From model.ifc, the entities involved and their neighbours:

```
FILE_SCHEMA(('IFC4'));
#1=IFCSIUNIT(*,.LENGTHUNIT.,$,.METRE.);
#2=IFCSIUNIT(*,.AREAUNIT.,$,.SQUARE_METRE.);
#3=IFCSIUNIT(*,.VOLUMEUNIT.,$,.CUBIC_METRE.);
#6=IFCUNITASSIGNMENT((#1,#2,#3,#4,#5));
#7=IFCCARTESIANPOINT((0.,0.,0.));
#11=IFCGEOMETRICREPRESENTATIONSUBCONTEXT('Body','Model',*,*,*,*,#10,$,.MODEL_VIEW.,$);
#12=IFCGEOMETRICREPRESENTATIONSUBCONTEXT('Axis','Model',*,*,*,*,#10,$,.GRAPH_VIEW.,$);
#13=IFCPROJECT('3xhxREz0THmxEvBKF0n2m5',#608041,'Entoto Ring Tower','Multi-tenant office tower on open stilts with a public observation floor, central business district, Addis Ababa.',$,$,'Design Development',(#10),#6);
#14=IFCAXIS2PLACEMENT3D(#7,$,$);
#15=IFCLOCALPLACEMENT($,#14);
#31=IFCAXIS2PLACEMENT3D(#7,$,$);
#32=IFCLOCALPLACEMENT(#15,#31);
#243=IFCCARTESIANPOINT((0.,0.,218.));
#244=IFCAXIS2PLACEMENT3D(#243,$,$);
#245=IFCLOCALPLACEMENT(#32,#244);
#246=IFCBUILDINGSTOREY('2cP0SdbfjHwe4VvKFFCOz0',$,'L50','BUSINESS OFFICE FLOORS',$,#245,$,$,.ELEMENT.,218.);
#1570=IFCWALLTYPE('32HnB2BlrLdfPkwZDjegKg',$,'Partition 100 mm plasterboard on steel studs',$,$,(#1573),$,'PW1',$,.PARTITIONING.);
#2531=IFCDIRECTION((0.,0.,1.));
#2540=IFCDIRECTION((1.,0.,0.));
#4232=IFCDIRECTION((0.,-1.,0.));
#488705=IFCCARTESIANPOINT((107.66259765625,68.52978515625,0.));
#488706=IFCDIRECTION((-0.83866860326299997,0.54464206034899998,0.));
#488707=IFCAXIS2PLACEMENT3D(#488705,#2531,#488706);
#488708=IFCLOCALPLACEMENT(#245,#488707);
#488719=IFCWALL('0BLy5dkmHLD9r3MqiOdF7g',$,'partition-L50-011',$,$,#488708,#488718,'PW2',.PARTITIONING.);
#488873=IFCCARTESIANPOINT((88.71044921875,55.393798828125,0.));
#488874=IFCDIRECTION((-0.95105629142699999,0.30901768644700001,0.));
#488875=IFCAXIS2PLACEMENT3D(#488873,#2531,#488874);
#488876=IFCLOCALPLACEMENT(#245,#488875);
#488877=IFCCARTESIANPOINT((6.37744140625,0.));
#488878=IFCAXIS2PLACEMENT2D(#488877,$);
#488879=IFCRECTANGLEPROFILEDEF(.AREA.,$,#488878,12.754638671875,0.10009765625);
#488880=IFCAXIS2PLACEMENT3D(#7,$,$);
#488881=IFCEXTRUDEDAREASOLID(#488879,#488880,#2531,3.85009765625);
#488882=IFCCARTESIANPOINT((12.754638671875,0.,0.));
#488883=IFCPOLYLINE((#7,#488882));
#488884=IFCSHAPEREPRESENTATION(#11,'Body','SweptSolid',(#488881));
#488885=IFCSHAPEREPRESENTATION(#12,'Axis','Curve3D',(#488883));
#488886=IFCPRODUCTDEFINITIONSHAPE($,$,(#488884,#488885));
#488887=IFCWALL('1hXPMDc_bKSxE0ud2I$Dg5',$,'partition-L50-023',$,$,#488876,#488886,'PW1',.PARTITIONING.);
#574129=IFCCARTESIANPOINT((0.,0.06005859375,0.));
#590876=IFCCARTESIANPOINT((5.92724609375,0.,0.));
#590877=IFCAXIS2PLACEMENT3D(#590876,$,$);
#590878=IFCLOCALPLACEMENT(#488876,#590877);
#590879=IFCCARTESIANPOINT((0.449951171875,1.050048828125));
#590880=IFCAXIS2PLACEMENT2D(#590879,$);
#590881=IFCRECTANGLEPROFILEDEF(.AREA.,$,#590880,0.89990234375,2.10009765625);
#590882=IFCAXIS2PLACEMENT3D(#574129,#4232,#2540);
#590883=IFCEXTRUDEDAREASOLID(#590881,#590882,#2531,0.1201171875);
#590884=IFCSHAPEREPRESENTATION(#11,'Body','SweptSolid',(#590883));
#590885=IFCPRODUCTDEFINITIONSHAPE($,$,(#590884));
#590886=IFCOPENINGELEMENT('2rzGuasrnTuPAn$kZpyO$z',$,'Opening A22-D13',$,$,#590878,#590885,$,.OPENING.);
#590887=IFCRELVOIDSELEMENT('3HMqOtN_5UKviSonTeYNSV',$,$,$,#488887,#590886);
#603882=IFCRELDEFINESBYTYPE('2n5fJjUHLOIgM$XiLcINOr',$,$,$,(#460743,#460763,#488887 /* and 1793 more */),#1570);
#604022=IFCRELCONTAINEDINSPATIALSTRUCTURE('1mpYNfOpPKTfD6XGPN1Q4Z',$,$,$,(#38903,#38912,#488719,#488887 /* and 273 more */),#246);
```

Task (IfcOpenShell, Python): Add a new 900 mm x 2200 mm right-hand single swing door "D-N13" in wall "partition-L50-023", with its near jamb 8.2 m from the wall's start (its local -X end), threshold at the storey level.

```python
import numpy as np
import ifcopenshell
import ifcopenshell.api.feature
import ifcopenshell.api.geometry
import ifcopenshell.api.root
import ifcopenshell.api.spatial
import ifcopenshell.geom
import ifcopenshell.util.element
import ifcopenshell.util.placement
import ifcopenshell.util.representation
import ifcopenshell.util.shape
import ifcopenshell.util.unit

model = ifcopenshell.open("model.ifc")
unit_scale = ifcopenshell.util.unit.calculate_unit_scale(model)
settings = ifcopenshell.geom.settings()


def volume(element):
    """Net volume in cubic metres, openings subtracted."""
    shape = ifcopenshell.geom.create_shape(settings, element)
    return ifcopenshell.util.shape.get_volume(shape.geometry)


wall = model.by_guid("1hXPMDc_bKSxE0ud2I$Dg5")
storey = ifcopenshell.util.element.get_container(wall, ifc_class="IfcBuildingStorey")
context = ifcopenshell.util.representation.get_context(model, "Model", "Body", "MODEL_VIEW")
before = volume(wall)

width, height, from_end, sill = 0.9, 2.2, 8.2, 0.0  # metres

# The wall runs along its own X axis, and the end named is its -X end.
wall_shape = ifcopenshell.geom.create_shape(settings, wall)
x, y, z = ifcopenshell.util.shape.get_vertices(wall_shape.geometry).T
start = x.min() + from_end
face, thickness = float(y.min()), float(y.max() - y.min())
wall_matrix = ifcopenshell.util.placement.get_local_placement(wall.ObjectPlacement)
level = ifcopenshell.util.placement.get_local_placement(storey.ObjectPlacement)[2, 3]


def in_wall(x, y):
    """Placement at x, y metres in the wall's axes, at sill height."""
    matrix = wall_matrix.copy()
    matrix[:, 3] = wall_matrix @ np.array([x / unit_scale, y / unit_scale, 0.0, 1.0])
    matrix[2, 3] = level + sill / unit_scale
    return matrix


# Opening: a box that overshoots both wall faces by 50 mm.
opening = ifcopenshell.api.root.create_entity(model, ifc_class="IfcOpeningElement", predefined_type="OPENING")
box = ifcopenshell.api.geometry.add_wall_representation(
    model, context=context, length=width, height=height, thickness=thickness + 0.1
)
ifcopenshell.api.geometry.assign_representation(model, product=opening, representation=box)
ifcopenshell.api.geometry.edit_object_placement(model, product=opening, matrix=in_wall(start, face - 0.05), is_si=False)
ifcopenshell.api.feature.add_feature(model, feature=opening, element=wall)

door = ifcopenshell.api.root.create_entity(model, ifc_class="IfcDoor", name="D-N13", predefined_type="DOOR")
door.OverallWidth, door.OverallHeight = width / unit_scale, height / unit_scale
door.OperationType = "SINGLE_SWING_RIGHT"
body = ifcopenshell.api.geometry.add_door_representation(
    model,
    context=context,
    overall_width=door.OverallWidth,
    overall_height=door.OverallHeight,
    operation_type="SINGLE_SWING_RIGHT",
    lining_properties={"LiningDepth": thickness / unit_scale, "ThresholdDepth": thickness / unit_scale},
)
ifcopenshell.api.geometry.assign_representation(model, product=door, representation=body)
ifcopenshell.api.spatial.assign_container(model, products=[door], relating_structure=storey)
ifcopenshell.api.feature.add_filling(model, opening=opening, element=door)

# The lining spans the wall, so the door starts at the wall face.
ifcopenshell.api.geometry.edit_object_placement(model, product=door, matrix=in_wall(start, face), is_si=False)

after = volume(wall)

print(f"wall volume {before:.3f} -> {after:.3f} m3")

model.write("model_rev.ifc")
```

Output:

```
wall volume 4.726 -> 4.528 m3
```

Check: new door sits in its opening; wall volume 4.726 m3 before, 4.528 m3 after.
